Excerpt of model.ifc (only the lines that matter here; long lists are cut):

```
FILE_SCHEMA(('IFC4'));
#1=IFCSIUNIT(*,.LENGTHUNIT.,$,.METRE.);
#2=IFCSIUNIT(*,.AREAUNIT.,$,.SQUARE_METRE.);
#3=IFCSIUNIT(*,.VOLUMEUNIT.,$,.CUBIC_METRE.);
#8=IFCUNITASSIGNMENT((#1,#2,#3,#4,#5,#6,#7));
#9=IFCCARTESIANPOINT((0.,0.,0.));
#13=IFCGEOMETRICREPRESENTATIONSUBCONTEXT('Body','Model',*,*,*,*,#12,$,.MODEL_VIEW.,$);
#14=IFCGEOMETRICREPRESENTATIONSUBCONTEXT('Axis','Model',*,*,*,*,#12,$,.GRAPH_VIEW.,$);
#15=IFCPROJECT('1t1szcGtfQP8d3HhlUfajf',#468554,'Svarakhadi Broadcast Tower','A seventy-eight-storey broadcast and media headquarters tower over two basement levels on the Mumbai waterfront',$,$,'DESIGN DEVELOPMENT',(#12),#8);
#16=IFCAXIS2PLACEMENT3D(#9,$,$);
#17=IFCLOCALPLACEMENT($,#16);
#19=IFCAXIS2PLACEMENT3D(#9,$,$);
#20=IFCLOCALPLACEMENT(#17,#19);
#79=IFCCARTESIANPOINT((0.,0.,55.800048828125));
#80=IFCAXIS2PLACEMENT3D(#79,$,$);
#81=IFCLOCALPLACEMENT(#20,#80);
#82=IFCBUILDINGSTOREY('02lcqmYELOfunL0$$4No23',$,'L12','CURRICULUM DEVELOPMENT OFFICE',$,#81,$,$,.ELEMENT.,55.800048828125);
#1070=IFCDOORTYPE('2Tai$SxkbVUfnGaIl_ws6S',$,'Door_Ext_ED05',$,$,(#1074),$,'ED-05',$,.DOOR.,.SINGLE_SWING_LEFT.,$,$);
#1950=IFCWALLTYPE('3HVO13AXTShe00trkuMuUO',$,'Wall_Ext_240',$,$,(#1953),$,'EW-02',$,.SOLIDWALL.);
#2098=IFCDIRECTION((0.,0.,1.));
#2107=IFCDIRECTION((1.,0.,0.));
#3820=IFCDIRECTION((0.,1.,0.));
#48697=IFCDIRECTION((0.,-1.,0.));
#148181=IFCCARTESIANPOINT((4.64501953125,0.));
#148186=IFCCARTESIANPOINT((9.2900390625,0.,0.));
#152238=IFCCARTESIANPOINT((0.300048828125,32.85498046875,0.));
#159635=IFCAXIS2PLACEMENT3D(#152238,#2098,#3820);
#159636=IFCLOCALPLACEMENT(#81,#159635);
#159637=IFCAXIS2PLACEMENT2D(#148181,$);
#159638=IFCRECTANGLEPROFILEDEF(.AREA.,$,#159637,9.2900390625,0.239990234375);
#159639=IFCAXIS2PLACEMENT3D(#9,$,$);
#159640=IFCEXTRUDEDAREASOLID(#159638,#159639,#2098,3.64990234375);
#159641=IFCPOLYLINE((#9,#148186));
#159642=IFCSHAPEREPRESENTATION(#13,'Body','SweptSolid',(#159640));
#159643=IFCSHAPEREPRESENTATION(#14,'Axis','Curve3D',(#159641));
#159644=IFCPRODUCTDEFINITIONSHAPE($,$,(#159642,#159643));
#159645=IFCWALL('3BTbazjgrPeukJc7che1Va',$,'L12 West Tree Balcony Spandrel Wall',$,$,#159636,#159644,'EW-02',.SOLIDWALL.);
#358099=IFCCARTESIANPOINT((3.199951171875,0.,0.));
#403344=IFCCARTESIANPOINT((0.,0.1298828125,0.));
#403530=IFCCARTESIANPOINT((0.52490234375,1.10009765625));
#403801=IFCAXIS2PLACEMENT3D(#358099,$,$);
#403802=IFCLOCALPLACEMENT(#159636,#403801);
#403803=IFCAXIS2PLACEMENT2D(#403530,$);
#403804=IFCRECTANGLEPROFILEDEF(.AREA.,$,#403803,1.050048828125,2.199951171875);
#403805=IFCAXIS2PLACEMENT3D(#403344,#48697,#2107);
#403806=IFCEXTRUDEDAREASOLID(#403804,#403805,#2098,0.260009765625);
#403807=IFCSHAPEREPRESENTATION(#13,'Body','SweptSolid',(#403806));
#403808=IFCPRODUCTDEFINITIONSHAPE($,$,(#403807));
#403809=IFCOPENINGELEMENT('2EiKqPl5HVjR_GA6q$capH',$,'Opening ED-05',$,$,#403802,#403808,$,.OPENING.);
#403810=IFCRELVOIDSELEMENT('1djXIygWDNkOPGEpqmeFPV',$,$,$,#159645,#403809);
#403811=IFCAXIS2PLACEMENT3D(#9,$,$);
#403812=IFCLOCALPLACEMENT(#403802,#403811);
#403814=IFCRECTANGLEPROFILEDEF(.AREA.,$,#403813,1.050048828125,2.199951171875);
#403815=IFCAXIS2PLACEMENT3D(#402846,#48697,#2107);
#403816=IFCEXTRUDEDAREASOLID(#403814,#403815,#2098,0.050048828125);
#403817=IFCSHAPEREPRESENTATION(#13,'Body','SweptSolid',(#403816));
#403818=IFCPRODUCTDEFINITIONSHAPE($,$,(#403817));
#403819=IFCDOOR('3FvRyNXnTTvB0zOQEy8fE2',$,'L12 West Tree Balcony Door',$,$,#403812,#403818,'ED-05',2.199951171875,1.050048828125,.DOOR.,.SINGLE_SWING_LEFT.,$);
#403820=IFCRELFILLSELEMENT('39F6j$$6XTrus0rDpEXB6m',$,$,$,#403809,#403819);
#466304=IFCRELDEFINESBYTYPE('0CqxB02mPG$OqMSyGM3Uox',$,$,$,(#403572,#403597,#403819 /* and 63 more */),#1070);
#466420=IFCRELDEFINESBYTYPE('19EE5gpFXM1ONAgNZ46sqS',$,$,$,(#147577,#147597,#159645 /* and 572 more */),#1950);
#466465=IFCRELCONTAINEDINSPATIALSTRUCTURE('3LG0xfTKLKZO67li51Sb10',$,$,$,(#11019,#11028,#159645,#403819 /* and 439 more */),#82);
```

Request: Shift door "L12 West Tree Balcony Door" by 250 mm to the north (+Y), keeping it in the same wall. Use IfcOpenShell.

```python
import ifcopenshell
import ifcopenshell.api.geometry
import ifcopenshell.util.placement

model = ifcopenshell.open("model.ifc")

door = model.by_guid("3FvRyNXnTTvB0zOQEy8fE2")
opening = door.FillsVoids[0].RelatingOpeningElement
wall = opening.VoidsElements[0].RelatingBuildingElement

wall_matrix = ifcopenshell.util.placement.get_local_placement(wall.ObjectPlacement)
shift = wall_matrix[:3, 0] * 0.25
before = ifcopenshell.util.placement.get_local_placement(door.ObjectPlacement)[:3, 3].copy()

# The door is placed relative to its opening, so it follows when the opening moves.
matrix = ifcopenshell.util.placement.get_local_placement(opening.ObjectPlacement)
matrix[:3, 3] += shift
ifcopenshell.api.geometry.edit_object_placement(
    model, product=opening, matrix=matrix, is_si=False, should_transform_children=True
)

after = ifcopenshell.util.placement.get_local_placement(door.ObjectPlacement)[:3, 3]
print("door moved by", (after - before).round(3) + 0.0)

model.write("model_rev.ifc")
```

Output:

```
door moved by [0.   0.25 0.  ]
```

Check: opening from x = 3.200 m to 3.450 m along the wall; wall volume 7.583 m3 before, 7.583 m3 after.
